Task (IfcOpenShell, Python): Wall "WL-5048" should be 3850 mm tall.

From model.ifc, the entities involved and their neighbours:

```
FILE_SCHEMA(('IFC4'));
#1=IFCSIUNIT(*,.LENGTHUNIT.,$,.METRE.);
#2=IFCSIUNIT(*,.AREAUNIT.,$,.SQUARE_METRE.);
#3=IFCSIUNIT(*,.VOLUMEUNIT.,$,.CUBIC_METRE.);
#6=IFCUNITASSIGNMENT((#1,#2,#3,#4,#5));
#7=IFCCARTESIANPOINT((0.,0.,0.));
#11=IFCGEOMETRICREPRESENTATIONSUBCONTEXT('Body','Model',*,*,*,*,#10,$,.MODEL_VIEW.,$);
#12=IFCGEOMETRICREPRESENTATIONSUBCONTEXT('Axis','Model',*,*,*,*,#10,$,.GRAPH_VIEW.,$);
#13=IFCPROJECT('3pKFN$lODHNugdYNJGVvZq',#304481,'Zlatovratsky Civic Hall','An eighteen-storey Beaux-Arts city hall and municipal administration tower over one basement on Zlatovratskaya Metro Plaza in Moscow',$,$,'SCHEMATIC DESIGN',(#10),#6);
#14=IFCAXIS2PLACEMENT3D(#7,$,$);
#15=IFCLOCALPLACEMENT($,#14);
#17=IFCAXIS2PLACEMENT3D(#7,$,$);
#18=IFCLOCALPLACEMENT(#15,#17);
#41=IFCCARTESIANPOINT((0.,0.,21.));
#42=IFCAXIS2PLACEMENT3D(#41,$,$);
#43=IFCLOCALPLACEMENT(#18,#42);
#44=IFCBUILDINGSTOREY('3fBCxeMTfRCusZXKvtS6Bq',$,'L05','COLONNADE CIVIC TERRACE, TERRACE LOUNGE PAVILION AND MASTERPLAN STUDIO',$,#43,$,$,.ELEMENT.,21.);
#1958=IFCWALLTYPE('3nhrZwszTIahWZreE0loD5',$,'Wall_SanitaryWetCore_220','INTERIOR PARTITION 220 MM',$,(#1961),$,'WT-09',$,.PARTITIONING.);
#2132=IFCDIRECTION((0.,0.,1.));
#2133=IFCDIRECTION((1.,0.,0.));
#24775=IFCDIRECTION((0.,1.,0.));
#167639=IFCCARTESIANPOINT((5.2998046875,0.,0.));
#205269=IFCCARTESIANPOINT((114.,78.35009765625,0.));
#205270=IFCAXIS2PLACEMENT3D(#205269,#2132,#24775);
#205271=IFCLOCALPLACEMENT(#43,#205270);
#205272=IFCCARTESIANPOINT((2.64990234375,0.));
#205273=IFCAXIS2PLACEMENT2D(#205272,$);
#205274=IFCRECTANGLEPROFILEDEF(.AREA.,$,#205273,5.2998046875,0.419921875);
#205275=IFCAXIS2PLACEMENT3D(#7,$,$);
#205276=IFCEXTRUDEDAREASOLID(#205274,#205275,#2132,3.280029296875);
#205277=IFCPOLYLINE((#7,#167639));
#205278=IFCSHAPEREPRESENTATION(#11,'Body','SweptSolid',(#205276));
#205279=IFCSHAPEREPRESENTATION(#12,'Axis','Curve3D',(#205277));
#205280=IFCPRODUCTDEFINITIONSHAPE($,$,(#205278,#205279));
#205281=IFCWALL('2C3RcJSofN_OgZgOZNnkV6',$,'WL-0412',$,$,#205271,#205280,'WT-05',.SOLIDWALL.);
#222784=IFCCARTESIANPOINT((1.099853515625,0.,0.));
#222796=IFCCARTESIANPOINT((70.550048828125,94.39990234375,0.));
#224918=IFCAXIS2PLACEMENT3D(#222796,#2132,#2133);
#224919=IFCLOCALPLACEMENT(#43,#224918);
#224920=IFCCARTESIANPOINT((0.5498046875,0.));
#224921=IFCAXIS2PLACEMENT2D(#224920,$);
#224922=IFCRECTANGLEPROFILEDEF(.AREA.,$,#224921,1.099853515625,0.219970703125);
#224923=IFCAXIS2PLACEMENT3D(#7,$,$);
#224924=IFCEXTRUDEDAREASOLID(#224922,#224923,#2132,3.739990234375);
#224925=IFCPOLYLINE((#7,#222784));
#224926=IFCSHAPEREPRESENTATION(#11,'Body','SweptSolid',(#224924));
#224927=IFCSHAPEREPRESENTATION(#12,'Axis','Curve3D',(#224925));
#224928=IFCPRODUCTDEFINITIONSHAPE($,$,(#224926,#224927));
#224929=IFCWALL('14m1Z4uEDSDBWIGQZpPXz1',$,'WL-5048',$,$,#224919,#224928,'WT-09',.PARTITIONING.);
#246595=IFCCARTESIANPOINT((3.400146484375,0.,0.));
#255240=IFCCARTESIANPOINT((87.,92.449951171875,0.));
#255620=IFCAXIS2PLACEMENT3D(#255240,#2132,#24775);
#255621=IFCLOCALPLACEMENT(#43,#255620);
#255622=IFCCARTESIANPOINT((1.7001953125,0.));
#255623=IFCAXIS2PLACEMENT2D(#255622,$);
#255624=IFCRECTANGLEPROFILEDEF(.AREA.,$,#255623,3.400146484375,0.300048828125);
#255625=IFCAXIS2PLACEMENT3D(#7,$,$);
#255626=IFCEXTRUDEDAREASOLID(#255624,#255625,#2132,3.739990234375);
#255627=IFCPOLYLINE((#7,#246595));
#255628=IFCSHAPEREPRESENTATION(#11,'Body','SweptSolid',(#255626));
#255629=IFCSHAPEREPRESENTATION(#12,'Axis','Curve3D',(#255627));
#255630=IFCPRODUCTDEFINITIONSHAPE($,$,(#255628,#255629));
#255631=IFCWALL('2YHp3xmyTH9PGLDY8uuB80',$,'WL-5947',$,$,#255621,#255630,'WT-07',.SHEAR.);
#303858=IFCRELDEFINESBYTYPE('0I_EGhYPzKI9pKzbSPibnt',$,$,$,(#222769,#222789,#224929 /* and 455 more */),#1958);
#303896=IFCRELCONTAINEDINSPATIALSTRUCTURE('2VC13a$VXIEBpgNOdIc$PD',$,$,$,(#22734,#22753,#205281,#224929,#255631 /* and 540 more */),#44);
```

```python
import ifcopenshell
import ifcopenshell.geom
import ifcopenshell.util.representation
import ifcopenshell.util.shape

model = ifcopenshell.open("model.ifc")
settings = ifcopenshell.geom.settings()


def volume(element):
    """Net volume in cubic metres, openings subtracted."""
    shape = ifcopenshell.geom.create_shape(settings, element)
    return ifcopenshell.util.shape.get_volume(shape.geometry)


wall = model.by_id(224929)
before = volume(wall)

body = ifcopenshell.util.representation.get_representation(wall, "Model", "Body")
solid = body.Items[0]
old_height = solid.Depth
solid.Depth = 3.85
after = volume(wall)

print(f"height {old_height:g} -> {solid.Depth:g}, volume {before:.3f} -> {after:.3f} m3")

model.write("model_updated.ifc")
```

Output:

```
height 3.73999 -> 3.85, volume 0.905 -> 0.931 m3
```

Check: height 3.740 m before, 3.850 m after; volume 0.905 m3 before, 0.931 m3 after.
